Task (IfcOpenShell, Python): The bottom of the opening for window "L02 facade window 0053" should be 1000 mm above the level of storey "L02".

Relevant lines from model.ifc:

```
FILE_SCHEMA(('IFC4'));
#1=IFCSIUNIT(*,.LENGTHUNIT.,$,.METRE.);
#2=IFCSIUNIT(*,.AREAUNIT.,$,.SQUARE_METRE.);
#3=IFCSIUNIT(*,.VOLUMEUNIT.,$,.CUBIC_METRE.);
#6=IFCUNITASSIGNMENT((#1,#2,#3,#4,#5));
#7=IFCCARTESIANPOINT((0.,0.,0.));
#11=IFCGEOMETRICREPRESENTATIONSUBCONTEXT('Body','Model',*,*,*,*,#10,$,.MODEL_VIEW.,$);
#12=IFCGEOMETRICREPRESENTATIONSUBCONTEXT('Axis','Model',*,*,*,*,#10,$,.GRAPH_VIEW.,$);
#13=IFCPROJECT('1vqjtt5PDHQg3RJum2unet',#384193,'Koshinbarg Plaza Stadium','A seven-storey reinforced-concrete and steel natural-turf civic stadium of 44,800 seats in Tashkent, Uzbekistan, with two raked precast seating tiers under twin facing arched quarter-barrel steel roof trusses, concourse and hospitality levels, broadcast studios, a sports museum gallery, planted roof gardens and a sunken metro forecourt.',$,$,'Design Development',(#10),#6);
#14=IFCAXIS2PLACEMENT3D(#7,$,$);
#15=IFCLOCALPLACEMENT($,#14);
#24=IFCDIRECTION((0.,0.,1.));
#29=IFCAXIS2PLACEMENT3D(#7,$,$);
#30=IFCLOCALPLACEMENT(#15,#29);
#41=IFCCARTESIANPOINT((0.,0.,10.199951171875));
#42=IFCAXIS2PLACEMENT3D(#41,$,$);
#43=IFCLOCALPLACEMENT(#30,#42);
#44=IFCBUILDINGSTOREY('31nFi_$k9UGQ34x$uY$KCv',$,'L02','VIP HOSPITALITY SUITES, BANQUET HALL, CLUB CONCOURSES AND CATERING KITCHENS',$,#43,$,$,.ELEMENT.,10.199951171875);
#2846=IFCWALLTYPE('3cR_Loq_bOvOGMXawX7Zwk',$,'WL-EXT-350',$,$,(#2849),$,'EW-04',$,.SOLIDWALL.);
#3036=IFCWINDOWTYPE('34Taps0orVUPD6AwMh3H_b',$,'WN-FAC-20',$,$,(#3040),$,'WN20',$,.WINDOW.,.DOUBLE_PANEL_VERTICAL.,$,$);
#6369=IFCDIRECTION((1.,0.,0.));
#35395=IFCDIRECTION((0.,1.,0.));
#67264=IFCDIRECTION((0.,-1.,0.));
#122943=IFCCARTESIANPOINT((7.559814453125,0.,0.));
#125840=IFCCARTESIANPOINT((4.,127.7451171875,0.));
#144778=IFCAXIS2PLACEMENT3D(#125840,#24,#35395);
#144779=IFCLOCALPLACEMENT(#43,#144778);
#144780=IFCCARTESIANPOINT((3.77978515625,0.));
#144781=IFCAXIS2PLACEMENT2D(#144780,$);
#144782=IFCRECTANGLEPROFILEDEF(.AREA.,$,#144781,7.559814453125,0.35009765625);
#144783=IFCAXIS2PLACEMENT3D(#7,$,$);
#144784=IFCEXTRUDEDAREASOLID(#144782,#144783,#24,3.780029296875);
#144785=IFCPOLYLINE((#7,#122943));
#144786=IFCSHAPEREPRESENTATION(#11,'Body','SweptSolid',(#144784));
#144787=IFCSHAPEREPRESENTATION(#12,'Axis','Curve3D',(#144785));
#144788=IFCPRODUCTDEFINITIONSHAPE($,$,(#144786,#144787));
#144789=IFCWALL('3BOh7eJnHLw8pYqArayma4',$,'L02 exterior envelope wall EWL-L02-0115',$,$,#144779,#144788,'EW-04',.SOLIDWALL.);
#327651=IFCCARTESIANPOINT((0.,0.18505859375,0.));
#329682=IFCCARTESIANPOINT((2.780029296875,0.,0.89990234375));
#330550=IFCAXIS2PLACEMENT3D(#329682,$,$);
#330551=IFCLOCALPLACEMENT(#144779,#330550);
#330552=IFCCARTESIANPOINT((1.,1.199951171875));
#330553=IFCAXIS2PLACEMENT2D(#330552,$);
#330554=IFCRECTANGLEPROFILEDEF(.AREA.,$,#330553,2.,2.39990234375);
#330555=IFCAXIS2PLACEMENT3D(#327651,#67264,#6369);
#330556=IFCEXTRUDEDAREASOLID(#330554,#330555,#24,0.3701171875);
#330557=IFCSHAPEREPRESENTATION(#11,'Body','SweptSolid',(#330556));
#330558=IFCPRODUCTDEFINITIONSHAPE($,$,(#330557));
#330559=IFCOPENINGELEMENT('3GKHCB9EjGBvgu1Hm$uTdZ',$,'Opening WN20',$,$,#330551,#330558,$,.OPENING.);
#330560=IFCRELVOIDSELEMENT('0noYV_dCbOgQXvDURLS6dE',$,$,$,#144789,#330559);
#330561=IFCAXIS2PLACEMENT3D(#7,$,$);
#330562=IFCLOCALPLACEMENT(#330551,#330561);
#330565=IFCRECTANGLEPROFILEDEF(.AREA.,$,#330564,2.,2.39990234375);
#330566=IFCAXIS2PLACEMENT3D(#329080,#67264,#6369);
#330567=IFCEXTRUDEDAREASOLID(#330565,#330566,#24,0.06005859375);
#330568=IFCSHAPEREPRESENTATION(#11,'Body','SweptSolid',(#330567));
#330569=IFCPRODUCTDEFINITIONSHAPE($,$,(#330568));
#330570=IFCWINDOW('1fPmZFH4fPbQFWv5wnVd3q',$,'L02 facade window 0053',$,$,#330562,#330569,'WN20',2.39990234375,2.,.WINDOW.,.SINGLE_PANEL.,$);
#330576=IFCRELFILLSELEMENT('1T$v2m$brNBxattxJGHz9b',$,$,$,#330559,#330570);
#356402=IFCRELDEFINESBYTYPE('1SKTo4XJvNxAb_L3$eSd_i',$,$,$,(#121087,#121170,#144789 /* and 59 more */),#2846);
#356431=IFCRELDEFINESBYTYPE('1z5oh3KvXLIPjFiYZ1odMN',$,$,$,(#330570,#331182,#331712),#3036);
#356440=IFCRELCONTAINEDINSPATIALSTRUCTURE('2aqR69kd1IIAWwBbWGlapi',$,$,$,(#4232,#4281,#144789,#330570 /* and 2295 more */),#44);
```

```python
import numpy as np
import ifcopenshell
import ifcopenshell.api.geometry
import ifcopenshell.geom
import ifcopenshell.util.element
import ifcopenshell.util.placement
import ifcopenshell.util.shape
import ifcopenshell.util.unit

model = ifcopenshell.open("model.ifc")
unit_scale = ifcopenshell.util.unit.calculate_unit_scale(model)

window = model.by_guid("1fPmZFH4fPbQFWv5wnVd3q")
opening = window.FillsVoids[0].RelatingOpeningElement
storey = ifcopenshell.util.element.get_container(window, ifc_class="IfcBuildingStorey")
level = ifcopenshell.util.placement.get_local_placement(storey.ObjectPlacement)[2, 3]

# The opening's origin need not be at the sill, so measure its lowest point.
shape = ifcopenshell.geom.create_shape(ifcopenshell.geom.settings(), opening)
bottom = ifcopenshell.util.shape.get_shape_bottom_elevation(shape, shape.geometry) / unit_scale
dz = level + 1 / unit_scale - bottom

shift = np.array([0.0, 0.0, dz])
# The window is placed relative to its opening, so it follows when the opening moves.
matrix = ifcopenshell.util.placement.get_local_placement(opening.ObjectPlacement)
matrix[:3, 3] += shift
ifcopenshell.api.geometry.edit_object_placement(
    model, product=opening, matrix=matrix, is_si=False, should_transform_children=True
)

print(f"moved by {dz * unit_scale:+.3f} m")

model.write("model_updated.ifc")
```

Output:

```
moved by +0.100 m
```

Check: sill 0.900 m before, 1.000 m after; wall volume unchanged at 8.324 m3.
